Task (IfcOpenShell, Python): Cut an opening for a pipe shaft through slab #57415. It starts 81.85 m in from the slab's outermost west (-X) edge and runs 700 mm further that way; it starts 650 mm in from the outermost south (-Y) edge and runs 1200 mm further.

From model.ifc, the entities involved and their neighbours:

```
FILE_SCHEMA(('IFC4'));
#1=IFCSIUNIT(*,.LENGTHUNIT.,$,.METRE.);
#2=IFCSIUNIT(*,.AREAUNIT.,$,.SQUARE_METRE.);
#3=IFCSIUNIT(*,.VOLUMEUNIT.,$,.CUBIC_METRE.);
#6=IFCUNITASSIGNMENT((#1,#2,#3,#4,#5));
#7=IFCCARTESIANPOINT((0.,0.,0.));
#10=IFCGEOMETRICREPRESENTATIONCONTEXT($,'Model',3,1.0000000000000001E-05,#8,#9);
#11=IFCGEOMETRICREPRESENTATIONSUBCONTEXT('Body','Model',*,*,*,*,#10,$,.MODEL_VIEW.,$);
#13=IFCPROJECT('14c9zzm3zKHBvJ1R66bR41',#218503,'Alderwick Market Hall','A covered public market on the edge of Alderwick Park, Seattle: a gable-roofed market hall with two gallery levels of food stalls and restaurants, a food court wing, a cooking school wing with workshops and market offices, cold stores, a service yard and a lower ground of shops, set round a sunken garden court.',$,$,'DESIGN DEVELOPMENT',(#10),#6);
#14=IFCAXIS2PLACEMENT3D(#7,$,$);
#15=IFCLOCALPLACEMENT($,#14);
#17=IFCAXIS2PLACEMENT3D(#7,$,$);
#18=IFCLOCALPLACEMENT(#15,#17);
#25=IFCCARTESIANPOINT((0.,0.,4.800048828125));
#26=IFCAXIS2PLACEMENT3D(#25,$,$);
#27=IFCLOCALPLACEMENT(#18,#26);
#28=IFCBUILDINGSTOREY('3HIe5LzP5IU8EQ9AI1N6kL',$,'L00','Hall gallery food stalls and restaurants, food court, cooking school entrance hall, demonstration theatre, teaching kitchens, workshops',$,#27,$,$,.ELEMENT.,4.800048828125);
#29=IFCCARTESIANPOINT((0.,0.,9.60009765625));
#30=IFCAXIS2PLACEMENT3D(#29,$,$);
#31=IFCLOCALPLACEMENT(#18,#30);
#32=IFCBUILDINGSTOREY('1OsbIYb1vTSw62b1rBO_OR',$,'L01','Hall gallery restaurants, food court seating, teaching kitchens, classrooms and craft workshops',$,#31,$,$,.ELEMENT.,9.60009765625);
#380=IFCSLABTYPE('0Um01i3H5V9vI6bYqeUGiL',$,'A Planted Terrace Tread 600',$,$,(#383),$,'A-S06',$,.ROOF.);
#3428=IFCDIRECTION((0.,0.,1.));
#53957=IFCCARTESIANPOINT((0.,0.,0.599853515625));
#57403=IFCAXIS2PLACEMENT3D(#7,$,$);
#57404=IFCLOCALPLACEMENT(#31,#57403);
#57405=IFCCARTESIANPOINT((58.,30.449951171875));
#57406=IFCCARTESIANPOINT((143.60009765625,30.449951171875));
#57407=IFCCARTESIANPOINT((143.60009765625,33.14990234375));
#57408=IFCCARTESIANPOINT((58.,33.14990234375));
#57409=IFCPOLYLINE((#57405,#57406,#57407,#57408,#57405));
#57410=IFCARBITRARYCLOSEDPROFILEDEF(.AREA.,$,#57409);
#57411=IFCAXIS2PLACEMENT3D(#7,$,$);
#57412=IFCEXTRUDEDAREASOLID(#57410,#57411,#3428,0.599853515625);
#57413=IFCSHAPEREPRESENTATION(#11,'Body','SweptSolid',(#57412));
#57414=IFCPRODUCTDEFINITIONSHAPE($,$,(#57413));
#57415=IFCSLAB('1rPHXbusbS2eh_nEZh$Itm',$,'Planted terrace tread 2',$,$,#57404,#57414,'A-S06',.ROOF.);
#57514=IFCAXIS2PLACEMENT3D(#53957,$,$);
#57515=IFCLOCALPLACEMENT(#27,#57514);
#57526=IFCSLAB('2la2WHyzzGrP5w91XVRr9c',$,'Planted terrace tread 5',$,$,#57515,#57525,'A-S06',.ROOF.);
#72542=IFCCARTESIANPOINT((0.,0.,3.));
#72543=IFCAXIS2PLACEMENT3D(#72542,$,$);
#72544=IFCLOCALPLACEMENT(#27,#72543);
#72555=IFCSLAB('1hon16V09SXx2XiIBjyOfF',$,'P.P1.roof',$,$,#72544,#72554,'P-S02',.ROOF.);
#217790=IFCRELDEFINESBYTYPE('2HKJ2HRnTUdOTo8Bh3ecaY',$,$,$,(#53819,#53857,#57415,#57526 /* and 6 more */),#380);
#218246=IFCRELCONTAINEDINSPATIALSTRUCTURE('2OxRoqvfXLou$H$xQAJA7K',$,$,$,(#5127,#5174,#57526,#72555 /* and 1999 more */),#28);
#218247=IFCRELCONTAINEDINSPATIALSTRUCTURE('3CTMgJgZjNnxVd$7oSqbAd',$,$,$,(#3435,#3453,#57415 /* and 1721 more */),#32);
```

```python
import numpy as np
import ifcopenshell
import ifcopenshell.api.feature
import ifcopenshell.api.geometry
import ifcopenshell.api.root
import ifcopenshell.geom
import ifcopenshell.util.placement
import ifcopenshell.util.representation
import ifcopenshell.util.shape
import ifcopenshell.util.unit

model = ifcopenshell.open("model.ifc")
unit_scale = ifcopenshell.util.unit.calculate_unit_scale(model)
settings = ifcopenshell.geom.settings()


def volume(element):
    """Net volume in cubic metres, openings subtracted."""
    shape = ifcopenshell.geom.create_shape(settings, element)
    return ifcopenshell.util.shape.get_volume(shape.geometry)


slab = model.by_id(57415)
before = volume(slab)

# Extent in the slab's own axes, in metres. The edges named are its -X and -Y sides.
slab_shape = ifcopenshell.geom.create_shape(settings, slab)
vertices = ifcopenshell.util.shape.get_vertices(slab_shape.geometry)
x_min, y_min, bottom = vertices.min(axis=0)
top = vertices[:, 2].max()

opening = ifcopenshell.api.root.create_entity(model, ifc_class="IfcOpeningElement", name="Pipe shaft opening", predefined_type="OPENING")
context = ifcopenshell.util.representation.get_context(model, "Model", "Body", "MODEL_VIEW")
width, depth = 0.7, 1.2
outline = [(0.0, 0.0), (width, 0.0), (width, depth), (0.0, depth), (0.0, 0.0)]
# Overshoot both faces by 50 mm so the cut is clean.
shape = ifcopenshell.api.geometry.add_slab_representation(
    model, context=context, depth=top - bottom + 0.1, polyline=outline
)
ifcopenshell.api.geometry.assign_representation(model, product=opening, representation=shape)

matrix = ifcopenshell.util.placement.get_local_placement(slab.ObjectPlacement)
matrix[:, 3] = matrix @ np.append(np.array([x_min + 81.85, y_min + 0.65, bottom - 0.05]) / unit_scale, 1.0)
ifcopenshell.api.geometry.edit_object_placement(model, product=opening, matrix=matrix, is_si=False)
ifcopenshell.api.feature.add_feature(model, feature=opening, element=slab)

after = volume(slab)

print(f"slab volume {before:.3f} -> {after:.3f} m3")

model.write("model-out.ifc")
```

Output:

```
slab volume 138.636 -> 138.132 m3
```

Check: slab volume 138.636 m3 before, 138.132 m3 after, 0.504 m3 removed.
